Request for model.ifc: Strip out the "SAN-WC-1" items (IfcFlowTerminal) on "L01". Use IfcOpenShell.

First a look at what the model holds.

```python
import ifcopenshell
import ifcopenshell.util.element

model = ifcopenshell.open("model.ifc")
print(model.schema)
storey = next(s for s in model.by_type("IfcBuildingStorey") if s.Name == "L01")
terminals = [e for e in ifcopenshell.util.element.get_decomposition(storey) if e.is_a("IfcFlowTerminal")]
seen = {}
for e in terminals:
    element_type = ifcopenshell.util.element.get_type(e)
    name = element_type.Name if element_type not in (None, e) else None
    seen[name] = seen.get(name, 0) + 1
for name, count in sorted(seen.items(), key=str):
    print(count, "x", name)
```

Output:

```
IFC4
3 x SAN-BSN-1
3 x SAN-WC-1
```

```python
import ifcopenshell
import ifcopenshell.api.root
import ifcopenshell.util.element

model = ifcopenshell.open("model.ifc")

storey = next(s for s in model.by_type("IfcBuildingStorey") if s.Name == "L01")
terminals = [e for e in ifcopenshell.util.element.get_decomposition(storey) if e.is_a("IfcFlowTerminal")]
targets = [e for e in terminals if (t := ifcopenshell.util.element.get_type(e)) not in (None, e) and t.Name == "SAN-WC-1"]

for e in targets:
    ifcopenshell.api.root.remove_product(model, product=e)
print(len(targets), "removed")

model.write("model_rev.ifc")
```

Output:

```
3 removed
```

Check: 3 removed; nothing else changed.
